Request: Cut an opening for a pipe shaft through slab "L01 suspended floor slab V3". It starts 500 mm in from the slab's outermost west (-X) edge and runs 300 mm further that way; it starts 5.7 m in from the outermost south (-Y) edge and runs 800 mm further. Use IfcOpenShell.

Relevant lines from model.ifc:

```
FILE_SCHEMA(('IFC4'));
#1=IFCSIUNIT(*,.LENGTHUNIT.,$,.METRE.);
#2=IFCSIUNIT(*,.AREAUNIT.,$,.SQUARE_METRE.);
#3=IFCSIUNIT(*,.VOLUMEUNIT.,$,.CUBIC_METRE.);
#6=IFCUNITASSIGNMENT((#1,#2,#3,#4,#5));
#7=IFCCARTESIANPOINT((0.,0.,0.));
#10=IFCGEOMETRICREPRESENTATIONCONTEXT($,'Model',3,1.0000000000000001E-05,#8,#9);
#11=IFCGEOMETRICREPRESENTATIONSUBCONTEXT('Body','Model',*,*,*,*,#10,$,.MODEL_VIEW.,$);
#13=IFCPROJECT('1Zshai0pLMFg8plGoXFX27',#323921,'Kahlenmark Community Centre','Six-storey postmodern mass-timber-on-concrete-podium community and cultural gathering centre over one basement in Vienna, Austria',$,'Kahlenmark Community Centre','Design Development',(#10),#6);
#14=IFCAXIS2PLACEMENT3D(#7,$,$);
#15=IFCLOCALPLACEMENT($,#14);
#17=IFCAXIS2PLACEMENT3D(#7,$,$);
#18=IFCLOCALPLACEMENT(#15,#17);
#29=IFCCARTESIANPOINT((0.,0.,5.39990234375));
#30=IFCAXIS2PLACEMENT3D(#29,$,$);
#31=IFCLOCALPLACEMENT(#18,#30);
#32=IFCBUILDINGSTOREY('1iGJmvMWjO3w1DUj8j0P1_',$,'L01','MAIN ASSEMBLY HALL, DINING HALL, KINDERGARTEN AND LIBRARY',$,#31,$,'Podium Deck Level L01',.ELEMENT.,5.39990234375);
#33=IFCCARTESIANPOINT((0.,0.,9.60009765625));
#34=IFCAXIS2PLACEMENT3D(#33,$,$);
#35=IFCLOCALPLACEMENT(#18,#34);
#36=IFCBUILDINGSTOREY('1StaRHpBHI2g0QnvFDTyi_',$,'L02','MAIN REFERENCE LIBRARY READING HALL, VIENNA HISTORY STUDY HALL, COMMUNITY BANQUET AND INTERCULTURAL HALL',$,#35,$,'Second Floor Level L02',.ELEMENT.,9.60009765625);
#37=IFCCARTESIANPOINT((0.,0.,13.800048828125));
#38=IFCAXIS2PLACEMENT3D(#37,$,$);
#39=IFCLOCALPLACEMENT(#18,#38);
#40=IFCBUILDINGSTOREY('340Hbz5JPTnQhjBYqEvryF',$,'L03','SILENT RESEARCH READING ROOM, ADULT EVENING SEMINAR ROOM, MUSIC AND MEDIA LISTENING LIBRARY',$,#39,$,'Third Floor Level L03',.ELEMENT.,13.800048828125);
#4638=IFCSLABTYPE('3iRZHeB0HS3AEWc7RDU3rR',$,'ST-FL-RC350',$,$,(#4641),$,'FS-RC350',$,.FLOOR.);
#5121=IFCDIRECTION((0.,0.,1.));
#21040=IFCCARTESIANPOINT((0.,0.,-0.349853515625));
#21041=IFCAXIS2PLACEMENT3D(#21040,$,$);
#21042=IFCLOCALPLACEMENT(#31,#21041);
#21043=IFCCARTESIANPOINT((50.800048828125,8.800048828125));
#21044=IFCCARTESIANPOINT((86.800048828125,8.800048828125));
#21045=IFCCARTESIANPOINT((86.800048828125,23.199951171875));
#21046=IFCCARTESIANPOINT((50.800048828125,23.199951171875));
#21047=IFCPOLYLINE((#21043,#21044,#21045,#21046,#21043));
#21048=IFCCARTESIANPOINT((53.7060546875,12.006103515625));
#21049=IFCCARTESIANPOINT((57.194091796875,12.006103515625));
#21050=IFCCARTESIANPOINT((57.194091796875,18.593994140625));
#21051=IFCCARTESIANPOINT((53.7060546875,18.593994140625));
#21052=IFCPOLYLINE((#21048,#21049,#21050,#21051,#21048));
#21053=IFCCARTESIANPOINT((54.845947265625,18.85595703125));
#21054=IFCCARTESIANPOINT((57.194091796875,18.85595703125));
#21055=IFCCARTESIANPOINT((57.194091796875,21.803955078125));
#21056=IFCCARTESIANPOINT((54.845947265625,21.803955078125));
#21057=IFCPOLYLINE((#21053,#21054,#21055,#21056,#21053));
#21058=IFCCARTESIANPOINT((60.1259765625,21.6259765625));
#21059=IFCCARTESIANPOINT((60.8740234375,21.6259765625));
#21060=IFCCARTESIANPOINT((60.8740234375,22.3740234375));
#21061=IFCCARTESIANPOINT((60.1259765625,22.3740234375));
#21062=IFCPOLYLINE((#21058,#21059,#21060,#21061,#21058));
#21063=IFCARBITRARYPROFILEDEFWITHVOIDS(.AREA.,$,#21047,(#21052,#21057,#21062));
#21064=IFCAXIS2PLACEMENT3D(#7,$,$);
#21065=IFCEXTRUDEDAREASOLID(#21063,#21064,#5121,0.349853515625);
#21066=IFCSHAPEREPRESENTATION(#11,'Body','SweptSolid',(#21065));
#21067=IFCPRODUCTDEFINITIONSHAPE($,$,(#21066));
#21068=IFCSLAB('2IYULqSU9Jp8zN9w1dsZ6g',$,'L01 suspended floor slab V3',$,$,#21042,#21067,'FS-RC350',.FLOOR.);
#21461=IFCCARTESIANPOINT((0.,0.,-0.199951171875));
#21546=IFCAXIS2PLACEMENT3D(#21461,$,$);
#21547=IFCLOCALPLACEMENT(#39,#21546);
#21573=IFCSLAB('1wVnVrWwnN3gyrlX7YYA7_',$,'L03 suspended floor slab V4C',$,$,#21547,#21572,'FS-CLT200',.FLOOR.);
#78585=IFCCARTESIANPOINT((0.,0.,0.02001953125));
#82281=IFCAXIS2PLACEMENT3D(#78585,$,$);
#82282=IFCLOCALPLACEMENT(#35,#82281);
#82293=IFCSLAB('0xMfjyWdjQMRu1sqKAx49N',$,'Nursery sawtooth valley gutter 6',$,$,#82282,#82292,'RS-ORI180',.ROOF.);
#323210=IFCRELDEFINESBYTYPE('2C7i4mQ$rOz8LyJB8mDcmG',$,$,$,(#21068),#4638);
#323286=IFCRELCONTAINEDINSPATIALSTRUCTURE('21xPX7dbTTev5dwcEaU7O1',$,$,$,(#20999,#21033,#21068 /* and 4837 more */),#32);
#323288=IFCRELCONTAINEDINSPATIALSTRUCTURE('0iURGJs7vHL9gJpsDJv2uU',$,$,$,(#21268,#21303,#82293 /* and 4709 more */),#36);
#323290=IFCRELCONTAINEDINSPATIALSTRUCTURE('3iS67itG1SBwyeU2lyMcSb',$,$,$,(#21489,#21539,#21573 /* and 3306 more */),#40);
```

```python
import numpy as np
import ifcopenshell
import ifcopenshell.api.feature
import ifcopenshell.api.geometry
import ifcopenshell.api.root
import ifcopenshell.geom
import ifcopenshell.util.placement
import ifcopenshell.util.representation
import ifcopenshell.util.shape
import ifcopenshell.util.unit

model = ifcopenshell.open("model.ifc")
unit_scale = ifcopenshell.util.unit.calculate_unit_scale(model)
settings = ifcopenshell.geom.settings()


def volume(element):
    """Net volume in cubic metres, openings subtracted."""
    shape = ifcopenshell.geom.create_shape(settings, element)
    return ifcopenshell.util.shape.get_volume(shape.geometry)


slab = model.by_guid("2IYULqSU9Jp8zN9w1dsZ6g")
before = volume(slab)

# Extent in the slab's own axes, in metres. The edges named are its -X and -Y sides.
slab_shape = ifcopenshell.geom.create_shape(settings, slab)
vertices = ifcopenshell.util.shape.get_vertices(slab_shape.geometry)
x_min, y_min, bottom = vertices.min(axis=0)
top = vertices[:, 2].max()

opening = ifcopenshell.api.root.create_entity(model, ifc_class="IfcOpeningElement", name="Pipe shaft opening", predefined_type="OPENING")
context = ifcopenshell.util.representation.get_context(model, "Model", "Body", "MODEL_VIEW")
width, depth = 0.3, 0.8
outline = [(0.0, 0.0), (width, 0.0), (width, depth), (0.0, depth), (0.0, 0.0)]
# Overshoot both faces by 50 mm so the cut is clean.
shape = ifcopenshell.api.geometry.add_slab_representation(
    model, context=context, depth=top - bottom + 0.1, polyline=outline
)
ifcopenshell.api.geometry.assign_representation(model, product=opening, representation=shape)

matrix = ifcopenshell.util.placement.get_local_placement(slab.ObjectPlacement)
matrix[:, 3] = matrix @ np.append(np.array([x_min + 0.5, y_min + 5.7, bottom - 0.05]) / unit_scale, 1.0)
ifcopenshell.api.geometry.edit_object_placement(model, product=opening, matrix=matrix, is_si=False)
ifcopenshell.api.feature.add_feature(model, feature=opening, element=slab)

after = volume(slab)

print(f"slab volume {before:.3f} -> {after:.3f} m3")

model.write("model_rev.ifc")
```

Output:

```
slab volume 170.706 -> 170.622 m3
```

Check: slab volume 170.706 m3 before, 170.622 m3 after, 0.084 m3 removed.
